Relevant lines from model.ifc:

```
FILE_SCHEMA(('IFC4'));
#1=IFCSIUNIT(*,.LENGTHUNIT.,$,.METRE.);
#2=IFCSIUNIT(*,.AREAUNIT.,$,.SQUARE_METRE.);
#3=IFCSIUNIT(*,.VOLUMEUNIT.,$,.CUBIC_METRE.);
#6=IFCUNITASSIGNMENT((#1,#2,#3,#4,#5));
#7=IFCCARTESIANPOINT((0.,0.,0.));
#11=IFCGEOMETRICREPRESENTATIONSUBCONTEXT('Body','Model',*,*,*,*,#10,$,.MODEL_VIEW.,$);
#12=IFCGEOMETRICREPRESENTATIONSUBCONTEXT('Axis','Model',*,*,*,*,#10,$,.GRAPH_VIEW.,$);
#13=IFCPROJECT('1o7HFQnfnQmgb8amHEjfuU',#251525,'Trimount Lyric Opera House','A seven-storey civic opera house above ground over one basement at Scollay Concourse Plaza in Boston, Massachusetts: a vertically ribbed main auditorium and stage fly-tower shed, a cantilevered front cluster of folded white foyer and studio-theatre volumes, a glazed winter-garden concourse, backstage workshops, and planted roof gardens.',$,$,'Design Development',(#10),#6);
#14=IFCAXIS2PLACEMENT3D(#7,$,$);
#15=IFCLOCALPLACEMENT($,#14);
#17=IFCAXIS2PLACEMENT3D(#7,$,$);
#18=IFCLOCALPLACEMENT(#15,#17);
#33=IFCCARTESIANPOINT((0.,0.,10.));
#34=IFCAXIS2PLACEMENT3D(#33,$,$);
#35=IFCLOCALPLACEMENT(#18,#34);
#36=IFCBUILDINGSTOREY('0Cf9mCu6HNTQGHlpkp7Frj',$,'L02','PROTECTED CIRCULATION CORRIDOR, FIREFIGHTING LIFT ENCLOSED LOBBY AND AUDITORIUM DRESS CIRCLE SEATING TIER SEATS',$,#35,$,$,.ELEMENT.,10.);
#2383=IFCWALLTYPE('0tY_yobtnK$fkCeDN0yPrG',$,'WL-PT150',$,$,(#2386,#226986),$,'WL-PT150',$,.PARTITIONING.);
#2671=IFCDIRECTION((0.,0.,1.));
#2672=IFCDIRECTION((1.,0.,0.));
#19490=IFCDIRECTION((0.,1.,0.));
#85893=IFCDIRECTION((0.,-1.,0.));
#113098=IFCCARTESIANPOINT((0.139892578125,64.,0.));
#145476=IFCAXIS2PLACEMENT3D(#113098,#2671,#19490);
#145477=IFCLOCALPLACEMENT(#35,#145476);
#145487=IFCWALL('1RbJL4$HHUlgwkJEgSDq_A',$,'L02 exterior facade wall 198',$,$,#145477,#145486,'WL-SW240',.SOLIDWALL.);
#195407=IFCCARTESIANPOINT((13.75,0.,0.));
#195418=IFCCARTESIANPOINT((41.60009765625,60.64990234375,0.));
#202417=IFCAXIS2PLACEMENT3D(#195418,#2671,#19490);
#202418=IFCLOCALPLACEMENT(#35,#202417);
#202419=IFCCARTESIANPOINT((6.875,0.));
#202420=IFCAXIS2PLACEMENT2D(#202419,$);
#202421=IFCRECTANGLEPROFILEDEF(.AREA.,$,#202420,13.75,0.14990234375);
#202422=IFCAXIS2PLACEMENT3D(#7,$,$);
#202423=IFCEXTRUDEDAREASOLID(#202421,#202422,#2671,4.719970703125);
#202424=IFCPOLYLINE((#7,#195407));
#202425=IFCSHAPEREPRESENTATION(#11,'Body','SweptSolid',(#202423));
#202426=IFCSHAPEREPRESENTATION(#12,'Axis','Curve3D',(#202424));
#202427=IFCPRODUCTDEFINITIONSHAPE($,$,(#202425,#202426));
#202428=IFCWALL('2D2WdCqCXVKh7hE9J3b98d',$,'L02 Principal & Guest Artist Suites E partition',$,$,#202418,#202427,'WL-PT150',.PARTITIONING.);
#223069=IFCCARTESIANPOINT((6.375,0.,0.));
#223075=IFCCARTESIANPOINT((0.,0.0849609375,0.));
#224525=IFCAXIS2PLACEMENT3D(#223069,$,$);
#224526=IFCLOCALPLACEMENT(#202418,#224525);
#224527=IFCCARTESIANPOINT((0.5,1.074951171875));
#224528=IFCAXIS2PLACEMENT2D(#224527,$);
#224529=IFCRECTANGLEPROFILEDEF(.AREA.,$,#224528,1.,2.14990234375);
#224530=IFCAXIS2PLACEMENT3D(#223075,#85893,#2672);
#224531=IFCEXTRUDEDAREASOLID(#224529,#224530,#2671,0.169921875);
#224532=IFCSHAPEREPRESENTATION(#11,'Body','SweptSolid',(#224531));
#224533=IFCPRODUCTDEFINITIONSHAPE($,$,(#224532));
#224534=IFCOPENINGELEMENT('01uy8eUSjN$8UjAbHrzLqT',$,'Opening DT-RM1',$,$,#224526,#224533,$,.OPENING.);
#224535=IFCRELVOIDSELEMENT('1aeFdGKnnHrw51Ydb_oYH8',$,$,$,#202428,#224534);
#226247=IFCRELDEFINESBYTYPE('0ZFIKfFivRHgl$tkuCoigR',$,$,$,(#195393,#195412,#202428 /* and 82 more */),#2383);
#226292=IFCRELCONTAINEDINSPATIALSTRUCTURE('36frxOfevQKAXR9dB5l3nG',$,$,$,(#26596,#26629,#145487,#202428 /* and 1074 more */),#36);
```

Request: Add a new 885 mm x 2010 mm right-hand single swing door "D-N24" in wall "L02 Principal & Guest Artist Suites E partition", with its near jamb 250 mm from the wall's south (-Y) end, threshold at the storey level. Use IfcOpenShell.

```python
import numpy as np
import ifcopenshell
import ifcopenshell.api.feature
import ifcopenshell.api.geometry
import ifcopenshell.api.root
import ifcopenshell.api.spatial
import ifcopenshell.geom
import ifcopenshell.util.element
import ifcopenshell.util.placement
import ifcopenshell.util.representation
import ifcopenshell.util.shape
import ifcopenshell.util.unit

model = ifcopenshell.open("model.ifc")
unit_scale = ifcopenshell.util.unit.calculate_unit_scale(model)
settings = ifcopenshell.geom.settings()


def volume(element):
    """Net volume in cubic metres, openings subtracted."""
    shape = ifcopenshell.geom.create_shape(settings, element)
    return ifcopenshell.util.shape.get_volume(shape.geometry)


wall = model.by_guid("2D2WdCqCXVKh7hE9J3b98d")
storey = ifcopenshell.util.element.get_container(wall, ifc_class="IfcBuildingStorey")
context = ifcopenshell.util.representation.get_context(model, "Model", "Body", "MODEL_VIEW")
before = volume(wall)

width, height, from_end, sill = 0.885, 2.01, 0.25, 0.0  # metres

# The wall runs along its own X axis, and the end named is its -X end.
wall_shape = ifcopenshell.geom.create_shape(settings, wall)
x, y, z = ifcopenshell.util.shape.get_vertices(wall_shape.geometry).T
start = x.min() + from_end
face, thickness = float(y.min()), float(y.max() - y.min())
wall_matrix = ifcopenshell.util.placement.get_local_placement(wall.ObjectPlacement)
level = ifcopenshell.util.placement.get_local_placement(storey.ObjectPlacement)[2, 3]


def in_wall(x, y):
    """Placement at x, y metres in the wall's axes, at sill height."""
    matrix = wall_matrix.copy()
    matrix[:, 3] = wall_matrix @ np.array([x / unit_scale, y / unit_scale, 0.0, 1.0])
    matrix[2, 3] = level + sill / unit_scale
    return matrix


# Opening: a box that overshoots both wall faces by 50 mm.
opening = ifcopenshell.api.root.create_entity(model, ifc_class="IfcOpeningElement", predefined_type="OPENING")
box = ifcopenshell.api.geometry.add_wall_representation(
    model, context=context, length=width, height=height, thickness=thickness + 0.1
)
ifcopenshell.api.geometry.assign_representation(model, product=opening, representation=box)
ifcopenshell.api.geometry.edit_object_placement(model, product=opening, matrix=in_wall(start, face - 0.05), is_si=False)
ifcopenshell.api.feature.add_feature(model, feature=opening, element=wall)

door = ifcopenshell.api.root.create_entity(model, ifc_class="IfcDoor", name="D-N24", predefined_type="DOOR")
door.OverallWidth, door.OverallHeight = width / unit_scale, height / unit_scale
door.OperationType = "SINGLE_SWING_RIGHT"
body = ifcopenshell.api.geometry.add_door_representation(
    model,
    context=context,
    overall_width=door.OverallWidth,
    overall_height=door.OverallHeight,
    operation_type="SINGLE_SWING_RIGHT",
    lining_properties={"LiningDepth": thickness / unit_scale, "ThresholdDepth": thickness / unit_scale},
)
ifcopenshell.api.geometry.assign_representation(model, product=door, representation=body)
ifcopenshell.api.spatial.assign_container(model, products=[door], relating_structure=storey)
ifcopenshell.api.feature.add_filling(model, opening=opening, element=door)

# The lining spans the wall, so the door starts at the wall face.
ifcopenshell.api.geometry.edit_object_placement(model, product=door, matrix=in_wall(start, face), is_si=False)

after = volume(wall)

print(f"wall volume {before:.3f} -> {after:.3f} m3")

model.write("model_rev.ifc")
```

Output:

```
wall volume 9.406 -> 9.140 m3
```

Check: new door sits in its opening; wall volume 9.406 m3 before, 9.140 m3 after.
